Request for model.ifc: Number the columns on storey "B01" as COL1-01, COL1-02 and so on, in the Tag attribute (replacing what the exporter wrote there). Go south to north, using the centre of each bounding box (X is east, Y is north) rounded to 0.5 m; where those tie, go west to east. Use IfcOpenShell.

First a look at what the model holds.

```python
import ifcopenshell
import ifcopenshell.util.element
import ifcopenshell.util.placement

model = ifcopenshell.open("model.ifc")
print(model.schema)
storey = next(s for s in model.by_type("IfcBuildingStorey") if s.Name == "B01")
columns = [e for e in ifcopenshell.util.element.get_decomposition(storey) if e.is_a("IfcColumn")]
for e in sorted(columns, key=lambda e: e.id()):
    origin = ifcopenshell.util.placement.get_local_placement(e.ObjectPlacement)[:3, 3]
    print(e.id(), e.Tag, e.Name, origin.round(2) + 0.0, sep=" | ")
```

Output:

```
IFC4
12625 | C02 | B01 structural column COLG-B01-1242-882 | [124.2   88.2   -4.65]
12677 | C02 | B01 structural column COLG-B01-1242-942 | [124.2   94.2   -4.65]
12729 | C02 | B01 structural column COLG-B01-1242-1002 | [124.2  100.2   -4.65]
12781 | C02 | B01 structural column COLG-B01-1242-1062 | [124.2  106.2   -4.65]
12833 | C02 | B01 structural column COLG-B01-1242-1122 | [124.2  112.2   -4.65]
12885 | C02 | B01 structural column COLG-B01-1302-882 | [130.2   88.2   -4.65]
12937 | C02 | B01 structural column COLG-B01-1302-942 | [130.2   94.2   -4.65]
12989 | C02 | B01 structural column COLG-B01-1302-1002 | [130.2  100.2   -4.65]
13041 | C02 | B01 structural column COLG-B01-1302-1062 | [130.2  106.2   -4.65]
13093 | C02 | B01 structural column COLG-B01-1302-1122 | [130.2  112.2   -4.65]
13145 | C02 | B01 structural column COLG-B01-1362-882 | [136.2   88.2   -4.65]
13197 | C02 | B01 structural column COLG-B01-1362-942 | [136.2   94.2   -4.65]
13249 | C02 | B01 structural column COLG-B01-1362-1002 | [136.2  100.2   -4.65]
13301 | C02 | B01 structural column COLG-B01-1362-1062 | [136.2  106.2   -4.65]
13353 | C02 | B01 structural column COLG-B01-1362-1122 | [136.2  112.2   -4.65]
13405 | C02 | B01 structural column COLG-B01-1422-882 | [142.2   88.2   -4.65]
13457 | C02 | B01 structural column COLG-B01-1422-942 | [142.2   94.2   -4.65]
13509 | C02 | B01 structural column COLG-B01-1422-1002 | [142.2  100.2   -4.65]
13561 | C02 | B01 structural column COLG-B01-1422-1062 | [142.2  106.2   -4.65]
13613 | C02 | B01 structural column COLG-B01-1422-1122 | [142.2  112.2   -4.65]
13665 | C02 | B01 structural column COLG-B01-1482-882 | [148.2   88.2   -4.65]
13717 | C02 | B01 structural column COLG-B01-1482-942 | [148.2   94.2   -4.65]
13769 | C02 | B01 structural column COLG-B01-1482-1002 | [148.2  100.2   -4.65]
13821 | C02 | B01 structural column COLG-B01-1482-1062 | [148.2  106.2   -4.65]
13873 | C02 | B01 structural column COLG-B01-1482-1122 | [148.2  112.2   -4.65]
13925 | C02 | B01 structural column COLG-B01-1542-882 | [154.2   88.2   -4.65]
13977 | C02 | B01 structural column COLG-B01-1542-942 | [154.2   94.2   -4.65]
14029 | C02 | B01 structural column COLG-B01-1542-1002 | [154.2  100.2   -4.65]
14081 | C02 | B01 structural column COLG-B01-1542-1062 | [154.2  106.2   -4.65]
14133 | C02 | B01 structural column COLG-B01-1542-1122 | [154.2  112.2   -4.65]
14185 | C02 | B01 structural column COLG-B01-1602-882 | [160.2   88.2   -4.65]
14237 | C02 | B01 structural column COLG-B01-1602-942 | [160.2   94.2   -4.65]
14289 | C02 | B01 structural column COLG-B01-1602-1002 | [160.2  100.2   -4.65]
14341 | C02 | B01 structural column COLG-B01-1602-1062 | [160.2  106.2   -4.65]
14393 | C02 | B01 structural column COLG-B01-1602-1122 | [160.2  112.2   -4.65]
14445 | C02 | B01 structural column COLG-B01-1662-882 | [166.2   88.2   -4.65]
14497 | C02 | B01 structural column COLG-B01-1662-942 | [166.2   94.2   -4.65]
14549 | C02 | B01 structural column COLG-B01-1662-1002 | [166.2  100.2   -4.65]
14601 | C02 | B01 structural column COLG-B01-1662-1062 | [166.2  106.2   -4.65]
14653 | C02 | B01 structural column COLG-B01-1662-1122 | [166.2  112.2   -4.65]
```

```python
import ifcopenshell
import ifcopenshell.geom
import ifcopenshell.util.element
import ifcopenshell.util.shape

model = ifcopenshell.open("model.ifc")
settings = ifcopenshell.geom.settings()
settings.set("use-world-coords", True)


def centre(element):
    shape = ifcopenshell.geom.create_shape(settings, element)
    return ifcopenshell.util.shape.get_bbox_centroid(shape.geometry)


storey = next(s for s in model.by_type("IfcBuildingStorey") if s.Name == "B01")
columns = [e for e in ifcopenshell.util.element.get_decomposition(storey) if e.is_a("IfcColumn")]

# Insertion points can sit at a corner or the storey origin, so sort by the geometry (in metres).
centres = {e: centre(e) for e in columns}
columns.sort(key=lambda e: (round(centres[e][1] / 0.5), centres[e][0]))

for i, e in enumerate(columns, start=1):
    number = f"COL1-{i:02d}"
    e.Tag = number
    print(e.id(), number)

model.write("model_rev.ifc")
```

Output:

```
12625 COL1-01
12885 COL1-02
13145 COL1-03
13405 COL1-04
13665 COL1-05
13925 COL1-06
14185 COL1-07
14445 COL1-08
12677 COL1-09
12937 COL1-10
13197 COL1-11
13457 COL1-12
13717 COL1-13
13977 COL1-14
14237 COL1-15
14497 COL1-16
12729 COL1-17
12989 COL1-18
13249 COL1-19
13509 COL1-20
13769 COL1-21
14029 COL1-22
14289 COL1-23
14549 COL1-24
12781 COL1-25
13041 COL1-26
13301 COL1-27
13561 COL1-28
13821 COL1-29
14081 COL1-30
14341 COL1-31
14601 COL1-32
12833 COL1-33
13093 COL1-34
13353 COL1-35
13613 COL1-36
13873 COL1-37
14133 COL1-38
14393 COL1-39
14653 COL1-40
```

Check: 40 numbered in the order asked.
